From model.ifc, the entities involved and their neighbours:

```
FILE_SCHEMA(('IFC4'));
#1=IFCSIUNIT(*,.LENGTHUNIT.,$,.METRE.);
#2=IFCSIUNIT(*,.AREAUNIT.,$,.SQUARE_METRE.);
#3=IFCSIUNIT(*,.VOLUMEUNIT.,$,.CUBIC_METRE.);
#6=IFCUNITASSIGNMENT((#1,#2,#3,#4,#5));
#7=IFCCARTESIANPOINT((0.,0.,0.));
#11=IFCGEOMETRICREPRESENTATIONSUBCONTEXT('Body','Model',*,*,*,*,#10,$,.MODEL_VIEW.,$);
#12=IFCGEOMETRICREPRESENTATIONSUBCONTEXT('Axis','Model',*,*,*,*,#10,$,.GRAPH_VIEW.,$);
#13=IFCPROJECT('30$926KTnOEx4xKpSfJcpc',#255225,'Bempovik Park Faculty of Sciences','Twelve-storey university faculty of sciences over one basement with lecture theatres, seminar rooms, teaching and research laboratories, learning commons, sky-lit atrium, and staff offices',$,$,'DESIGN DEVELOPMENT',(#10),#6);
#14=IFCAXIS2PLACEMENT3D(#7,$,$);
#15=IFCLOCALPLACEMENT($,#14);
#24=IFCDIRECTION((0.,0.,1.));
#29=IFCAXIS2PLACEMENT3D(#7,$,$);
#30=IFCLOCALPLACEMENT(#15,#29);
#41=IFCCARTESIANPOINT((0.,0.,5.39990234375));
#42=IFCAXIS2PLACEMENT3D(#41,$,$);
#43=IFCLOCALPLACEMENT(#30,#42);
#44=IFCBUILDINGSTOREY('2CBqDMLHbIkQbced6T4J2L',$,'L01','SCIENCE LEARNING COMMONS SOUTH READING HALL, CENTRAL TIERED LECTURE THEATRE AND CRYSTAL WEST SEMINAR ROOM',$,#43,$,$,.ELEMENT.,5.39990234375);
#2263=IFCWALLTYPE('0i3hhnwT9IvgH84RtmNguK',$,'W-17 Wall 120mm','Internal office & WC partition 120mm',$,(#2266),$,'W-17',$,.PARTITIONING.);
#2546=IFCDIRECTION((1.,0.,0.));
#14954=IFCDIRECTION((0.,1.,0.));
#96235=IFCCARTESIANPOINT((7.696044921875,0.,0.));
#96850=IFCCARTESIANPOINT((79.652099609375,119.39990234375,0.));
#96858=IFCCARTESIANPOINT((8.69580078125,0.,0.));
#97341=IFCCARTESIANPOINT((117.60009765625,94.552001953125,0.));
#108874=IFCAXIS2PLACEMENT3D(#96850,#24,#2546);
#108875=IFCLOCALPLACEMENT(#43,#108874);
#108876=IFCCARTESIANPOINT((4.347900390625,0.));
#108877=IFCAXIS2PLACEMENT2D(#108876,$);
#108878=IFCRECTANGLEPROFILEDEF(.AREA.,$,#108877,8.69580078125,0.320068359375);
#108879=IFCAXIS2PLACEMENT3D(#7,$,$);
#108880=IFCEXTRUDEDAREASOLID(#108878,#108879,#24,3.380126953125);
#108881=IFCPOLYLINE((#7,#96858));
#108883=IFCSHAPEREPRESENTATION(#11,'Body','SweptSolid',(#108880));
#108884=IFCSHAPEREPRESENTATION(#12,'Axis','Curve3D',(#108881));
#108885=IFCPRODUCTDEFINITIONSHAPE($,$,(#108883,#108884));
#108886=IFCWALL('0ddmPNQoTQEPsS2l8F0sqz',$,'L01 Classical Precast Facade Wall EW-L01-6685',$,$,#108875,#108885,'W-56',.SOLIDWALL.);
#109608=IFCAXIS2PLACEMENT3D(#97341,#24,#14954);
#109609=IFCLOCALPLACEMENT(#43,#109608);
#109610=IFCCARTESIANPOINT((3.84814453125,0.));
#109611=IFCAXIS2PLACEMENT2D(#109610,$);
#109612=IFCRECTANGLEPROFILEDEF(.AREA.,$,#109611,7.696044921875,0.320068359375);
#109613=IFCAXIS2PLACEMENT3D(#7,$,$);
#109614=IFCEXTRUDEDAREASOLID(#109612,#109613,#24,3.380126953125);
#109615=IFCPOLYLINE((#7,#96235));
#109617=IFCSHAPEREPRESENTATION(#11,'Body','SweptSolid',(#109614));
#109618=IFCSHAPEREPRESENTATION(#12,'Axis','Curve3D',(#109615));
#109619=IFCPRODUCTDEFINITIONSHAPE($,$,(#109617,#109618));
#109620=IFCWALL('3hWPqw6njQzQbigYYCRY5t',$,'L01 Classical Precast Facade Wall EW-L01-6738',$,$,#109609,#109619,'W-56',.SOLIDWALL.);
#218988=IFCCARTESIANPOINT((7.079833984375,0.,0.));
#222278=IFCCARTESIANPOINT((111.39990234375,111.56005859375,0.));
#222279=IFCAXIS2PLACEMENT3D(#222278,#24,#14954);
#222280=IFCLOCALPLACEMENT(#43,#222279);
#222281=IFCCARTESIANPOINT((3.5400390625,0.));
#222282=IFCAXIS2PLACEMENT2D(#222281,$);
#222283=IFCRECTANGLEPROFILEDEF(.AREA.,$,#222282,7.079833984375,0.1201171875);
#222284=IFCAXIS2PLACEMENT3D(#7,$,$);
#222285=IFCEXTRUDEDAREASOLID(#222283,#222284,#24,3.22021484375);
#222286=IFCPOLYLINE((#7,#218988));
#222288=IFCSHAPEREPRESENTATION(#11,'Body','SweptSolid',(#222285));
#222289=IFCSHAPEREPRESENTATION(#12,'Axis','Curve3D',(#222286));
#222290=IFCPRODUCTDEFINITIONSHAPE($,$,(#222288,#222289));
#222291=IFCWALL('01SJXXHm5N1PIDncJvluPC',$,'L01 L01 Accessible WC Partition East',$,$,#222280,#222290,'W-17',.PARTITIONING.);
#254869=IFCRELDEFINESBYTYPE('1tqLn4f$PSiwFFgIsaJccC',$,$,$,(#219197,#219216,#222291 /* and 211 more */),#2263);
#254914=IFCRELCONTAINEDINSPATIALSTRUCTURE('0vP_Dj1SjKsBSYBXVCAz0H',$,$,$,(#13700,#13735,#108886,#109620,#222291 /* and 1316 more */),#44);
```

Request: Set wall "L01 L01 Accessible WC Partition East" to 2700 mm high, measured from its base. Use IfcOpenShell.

```python
import ifcopenshell
import ifcopenshell.geom
import ifcopenshell.util.representation
import ifcopenshell.util.shape

model = ifcopenshell.open("model.ifc")
settings = ifcopenshell.geom.settings()


def volume(element):
    """Net volume in cubic metres, openings subtracted."""
    shape = ifcopenshell.geom.create_shape(settings, element)
    return ifcopenshell.util.shape.get_volume(shape.geometry)


wall = model.by_guid("01SJXXHm5N1PIDncJvluPC")
before = volume(wall)

body = ifcopenshell.util.representation.get_representation(wall, "Model", "Body")
solid = body.Items[0]
old_height = solid.Depth
solid.Depth = 2.7
after = volume(wall)

print(f"height {old_height:g} -> {solid.Depth:g}, volume {before:.3f} -> {after:.3f} m3")

model.write("model_rev.ifc")
```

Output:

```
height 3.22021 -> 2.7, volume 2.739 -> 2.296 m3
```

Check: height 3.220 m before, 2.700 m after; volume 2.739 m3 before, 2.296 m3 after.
